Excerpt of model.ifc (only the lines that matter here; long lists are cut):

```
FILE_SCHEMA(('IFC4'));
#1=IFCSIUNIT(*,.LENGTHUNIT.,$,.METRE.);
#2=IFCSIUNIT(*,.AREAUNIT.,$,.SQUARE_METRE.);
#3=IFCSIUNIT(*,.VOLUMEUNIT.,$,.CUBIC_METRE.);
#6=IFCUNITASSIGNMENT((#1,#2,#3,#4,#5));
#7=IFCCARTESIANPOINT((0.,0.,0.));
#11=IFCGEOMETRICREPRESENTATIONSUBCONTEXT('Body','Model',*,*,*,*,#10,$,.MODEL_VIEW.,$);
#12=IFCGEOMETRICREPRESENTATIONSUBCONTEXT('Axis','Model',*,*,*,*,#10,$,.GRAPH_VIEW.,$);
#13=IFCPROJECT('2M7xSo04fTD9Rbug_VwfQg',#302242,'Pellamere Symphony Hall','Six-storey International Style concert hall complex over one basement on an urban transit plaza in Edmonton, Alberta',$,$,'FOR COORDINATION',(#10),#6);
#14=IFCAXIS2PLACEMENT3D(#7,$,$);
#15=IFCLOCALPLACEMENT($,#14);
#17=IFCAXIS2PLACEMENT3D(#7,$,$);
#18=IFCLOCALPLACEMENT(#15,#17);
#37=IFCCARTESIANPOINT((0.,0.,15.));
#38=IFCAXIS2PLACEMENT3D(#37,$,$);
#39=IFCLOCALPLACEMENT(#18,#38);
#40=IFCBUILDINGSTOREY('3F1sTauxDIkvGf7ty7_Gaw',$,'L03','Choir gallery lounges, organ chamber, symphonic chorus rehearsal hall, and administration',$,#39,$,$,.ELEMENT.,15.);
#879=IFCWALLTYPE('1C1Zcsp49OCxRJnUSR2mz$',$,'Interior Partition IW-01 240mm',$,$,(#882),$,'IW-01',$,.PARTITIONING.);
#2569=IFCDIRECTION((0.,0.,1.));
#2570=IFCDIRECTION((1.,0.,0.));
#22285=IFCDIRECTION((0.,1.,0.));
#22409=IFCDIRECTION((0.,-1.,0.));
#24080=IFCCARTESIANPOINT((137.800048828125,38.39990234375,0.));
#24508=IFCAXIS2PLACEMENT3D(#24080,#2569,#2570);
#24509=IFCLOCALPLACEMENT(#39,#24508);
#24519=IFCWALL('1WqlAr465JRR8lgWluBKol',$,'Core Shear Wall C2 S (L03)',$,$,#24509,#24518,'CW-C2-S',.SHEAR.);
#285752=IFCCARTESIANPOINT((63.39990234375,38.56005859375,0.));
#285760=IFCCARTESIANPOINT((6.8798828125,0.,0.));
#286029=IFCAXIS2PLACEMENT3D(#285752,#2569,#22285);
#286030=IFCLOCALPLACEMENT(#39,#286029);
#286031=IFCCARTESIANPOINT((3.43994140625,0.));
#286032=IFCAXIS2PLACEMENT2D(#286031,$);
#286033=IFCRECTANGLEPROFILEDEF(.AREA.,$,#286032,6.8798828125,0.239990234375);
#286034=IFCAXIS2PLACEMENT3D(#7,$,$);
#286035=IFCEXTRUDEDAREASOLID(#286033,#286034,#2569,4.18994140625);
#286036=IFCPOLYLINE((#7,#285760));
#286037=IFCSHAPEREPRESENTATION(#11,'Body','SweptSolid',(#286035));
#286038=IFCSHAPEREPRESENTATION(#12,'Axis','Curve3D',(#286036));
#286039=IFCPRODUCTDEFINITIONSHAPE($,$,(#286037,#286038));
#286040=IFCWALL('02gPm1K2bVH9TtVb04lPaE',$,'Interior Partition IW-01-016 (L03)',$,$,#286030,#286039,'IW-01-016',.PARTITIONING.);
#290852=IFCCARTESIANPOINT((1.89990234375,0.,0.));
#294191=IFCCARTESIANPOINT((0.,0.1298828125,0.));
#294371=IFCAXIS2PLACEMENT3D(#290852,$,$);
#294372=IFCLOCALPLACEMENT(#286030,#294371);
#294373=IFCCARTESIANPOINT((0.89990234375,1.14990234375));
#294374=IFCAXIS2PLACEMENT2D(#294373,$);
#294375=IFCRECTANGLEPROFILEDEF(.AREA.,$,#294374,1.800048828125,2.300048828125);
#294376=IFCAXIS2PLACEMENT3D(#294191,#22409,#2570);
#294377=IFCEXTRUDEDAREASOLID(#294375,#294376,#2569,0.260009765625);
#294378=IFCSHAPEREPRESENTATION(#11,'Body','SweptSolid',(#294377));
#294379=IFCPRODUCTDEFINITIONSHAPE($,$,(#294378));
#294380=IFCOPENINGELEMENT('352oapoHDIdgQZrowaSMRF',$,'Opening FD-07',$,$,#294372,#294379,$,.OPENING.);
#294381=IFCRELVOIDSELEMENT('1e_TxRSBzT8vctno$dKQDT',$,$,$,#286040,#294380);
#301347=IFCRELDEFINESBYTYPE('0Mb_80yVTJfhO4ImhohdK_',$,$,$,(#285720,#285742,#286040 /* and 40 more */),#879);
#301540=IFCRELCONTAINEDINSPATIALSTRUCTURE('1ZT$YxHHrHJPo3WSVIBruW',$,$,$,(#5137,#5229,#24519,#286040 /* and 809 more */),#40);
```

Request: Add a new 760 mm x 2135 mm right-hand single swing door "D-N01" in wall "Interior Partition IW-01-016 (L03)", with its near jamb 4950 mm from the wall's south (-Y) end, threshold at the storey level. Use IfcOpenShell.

```python
import numpy as np
import ifcopenshell
import ifcopenshell.api.feature
import ifcopenshell.api.geometry
import ifcopenshell.api.root
import ifcopenshell.api.spatial
import ifcopenshell.geom
import ifcopenshell.util.element
import ifcopenshell.util.placement
import ifcopenshell.util.representation
import ifcopenshell.util.shape
import ifcopenshell.util.unit

model = ifcopenshell.open("model.ifc")
unit_scale = ifcopenshell.util.unit.calculate_unit_scale(model)
settings = ifcopenshell.geom.settings()


def volume(element):
    """Net volume in cubic metres, openings subtracted."""
    shape = ifcopenshell.geom.create_shape(settings, element)
    return ifcopenshell.util.shape.get_volume(shape.geometry)


wall = model.by_id(286040)
storey = ifcopenshell.util.element.get_container(wall, ifc_class="IfcBuildingStorey")
context = ifcopenshell.util.representation.get_context(model, "Model", "Body", "MODEL_VIEW")
before = volume(wall)

width, height, from_end, sill = 0.76, 2.135, 4.95, 0.0  # metres

# The wall runs along its own X axis, and the end named is its -X end.
wall_shape = ifcopenshell.geom.create_shape(settings, wall)
x, y, z = ifcopenshell.util.shape.get_vertices(wall_shape.geometry).T
start = x.min() + from_end
face, thickness = float(y.min()), float(y.max() - y.min())
wall_matrix = ifcopenshell.util.placement.get_local_placement(wall.ObjectPlacement)
level = ifcopenshell.util.placement.get_local_placement(storey.ObjectPlacement)[2, 3]


def in_wall(x, y):
    """Placement at x, y metres in the wall's axes, at sill height."""
    matrix = wall_matrix.copy()
    matrix[:, 3] = wall_matrix @ np.array([x / unit_scale, y / unit_scale, 0.0, 1.0])
    matrix[2, 3] = level + sill / unit_scale
    return matrix


# Opening: a box that overshoots both wall faces by 50 mm.
opening = ifcopenshell.api.root.create_entity(model, ifc_class="IfcOpeningElement", predefined_type="OPENING")
box = ifcopenshell.api.geometry.add_wall_representation(
    model, context=context, length=width, height=height, thickness=thickness + 0.1
)
ifcopenshell.api.geometry.assign_representation(model, product=opening, representation=box)
ifcopenshell.api.geometry.edit_object_placement(model, product=opening, matrix=in_wall(start, face - 0.05), is_si=False)
ifcopenshell.api.feature.add_feature(model, feature=opening, element=wall)

door = ifcopenshell.api.root.create_entity(model, ifc_class="IfcDoor", name="D-N01", predefined_type="DOOR")
door.OverallWidth, door.OverallHeight = width / unit_scale, height / unit_scale
door.OperationType = "SINGLE_SWING_RIGHT"
body = ifcopenshell.api.geometry.add_door_representation(
    model,
    context=context,
    overall_width=door.OverallWidth,
    overall_height=door.OverallHeight,
    operation_type="SINGLE_SWING_RIGHT",
    lining_properties={"LiningDepth": thickness / unit_scale, "ThresholdDepth": thickness / unit_scale},
)
ifcopenshell.api.geometry.assign_representation(model, product=door, representation=body)
ifcopenshell.api.spatial.assign_container(model, products=[door], relating_structure=storey)
ifcopenshell.api.feature.add_filling(model, opening=opening, element=door)

# The lining spans the wall, so the door starts at the wall face.
ifcopenshell.api.geometry.edit_object_placement(model, product=door, matrix=in_wall(start, face), is_si=False)

after = volume(wall)

print(f"wall volume {before:.3f} -> {after:.3f} m3")

model.write("model_updated.ifc")
```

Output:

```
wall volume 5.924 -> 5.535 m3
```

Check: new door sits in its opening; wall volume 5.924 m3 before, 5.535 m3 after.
